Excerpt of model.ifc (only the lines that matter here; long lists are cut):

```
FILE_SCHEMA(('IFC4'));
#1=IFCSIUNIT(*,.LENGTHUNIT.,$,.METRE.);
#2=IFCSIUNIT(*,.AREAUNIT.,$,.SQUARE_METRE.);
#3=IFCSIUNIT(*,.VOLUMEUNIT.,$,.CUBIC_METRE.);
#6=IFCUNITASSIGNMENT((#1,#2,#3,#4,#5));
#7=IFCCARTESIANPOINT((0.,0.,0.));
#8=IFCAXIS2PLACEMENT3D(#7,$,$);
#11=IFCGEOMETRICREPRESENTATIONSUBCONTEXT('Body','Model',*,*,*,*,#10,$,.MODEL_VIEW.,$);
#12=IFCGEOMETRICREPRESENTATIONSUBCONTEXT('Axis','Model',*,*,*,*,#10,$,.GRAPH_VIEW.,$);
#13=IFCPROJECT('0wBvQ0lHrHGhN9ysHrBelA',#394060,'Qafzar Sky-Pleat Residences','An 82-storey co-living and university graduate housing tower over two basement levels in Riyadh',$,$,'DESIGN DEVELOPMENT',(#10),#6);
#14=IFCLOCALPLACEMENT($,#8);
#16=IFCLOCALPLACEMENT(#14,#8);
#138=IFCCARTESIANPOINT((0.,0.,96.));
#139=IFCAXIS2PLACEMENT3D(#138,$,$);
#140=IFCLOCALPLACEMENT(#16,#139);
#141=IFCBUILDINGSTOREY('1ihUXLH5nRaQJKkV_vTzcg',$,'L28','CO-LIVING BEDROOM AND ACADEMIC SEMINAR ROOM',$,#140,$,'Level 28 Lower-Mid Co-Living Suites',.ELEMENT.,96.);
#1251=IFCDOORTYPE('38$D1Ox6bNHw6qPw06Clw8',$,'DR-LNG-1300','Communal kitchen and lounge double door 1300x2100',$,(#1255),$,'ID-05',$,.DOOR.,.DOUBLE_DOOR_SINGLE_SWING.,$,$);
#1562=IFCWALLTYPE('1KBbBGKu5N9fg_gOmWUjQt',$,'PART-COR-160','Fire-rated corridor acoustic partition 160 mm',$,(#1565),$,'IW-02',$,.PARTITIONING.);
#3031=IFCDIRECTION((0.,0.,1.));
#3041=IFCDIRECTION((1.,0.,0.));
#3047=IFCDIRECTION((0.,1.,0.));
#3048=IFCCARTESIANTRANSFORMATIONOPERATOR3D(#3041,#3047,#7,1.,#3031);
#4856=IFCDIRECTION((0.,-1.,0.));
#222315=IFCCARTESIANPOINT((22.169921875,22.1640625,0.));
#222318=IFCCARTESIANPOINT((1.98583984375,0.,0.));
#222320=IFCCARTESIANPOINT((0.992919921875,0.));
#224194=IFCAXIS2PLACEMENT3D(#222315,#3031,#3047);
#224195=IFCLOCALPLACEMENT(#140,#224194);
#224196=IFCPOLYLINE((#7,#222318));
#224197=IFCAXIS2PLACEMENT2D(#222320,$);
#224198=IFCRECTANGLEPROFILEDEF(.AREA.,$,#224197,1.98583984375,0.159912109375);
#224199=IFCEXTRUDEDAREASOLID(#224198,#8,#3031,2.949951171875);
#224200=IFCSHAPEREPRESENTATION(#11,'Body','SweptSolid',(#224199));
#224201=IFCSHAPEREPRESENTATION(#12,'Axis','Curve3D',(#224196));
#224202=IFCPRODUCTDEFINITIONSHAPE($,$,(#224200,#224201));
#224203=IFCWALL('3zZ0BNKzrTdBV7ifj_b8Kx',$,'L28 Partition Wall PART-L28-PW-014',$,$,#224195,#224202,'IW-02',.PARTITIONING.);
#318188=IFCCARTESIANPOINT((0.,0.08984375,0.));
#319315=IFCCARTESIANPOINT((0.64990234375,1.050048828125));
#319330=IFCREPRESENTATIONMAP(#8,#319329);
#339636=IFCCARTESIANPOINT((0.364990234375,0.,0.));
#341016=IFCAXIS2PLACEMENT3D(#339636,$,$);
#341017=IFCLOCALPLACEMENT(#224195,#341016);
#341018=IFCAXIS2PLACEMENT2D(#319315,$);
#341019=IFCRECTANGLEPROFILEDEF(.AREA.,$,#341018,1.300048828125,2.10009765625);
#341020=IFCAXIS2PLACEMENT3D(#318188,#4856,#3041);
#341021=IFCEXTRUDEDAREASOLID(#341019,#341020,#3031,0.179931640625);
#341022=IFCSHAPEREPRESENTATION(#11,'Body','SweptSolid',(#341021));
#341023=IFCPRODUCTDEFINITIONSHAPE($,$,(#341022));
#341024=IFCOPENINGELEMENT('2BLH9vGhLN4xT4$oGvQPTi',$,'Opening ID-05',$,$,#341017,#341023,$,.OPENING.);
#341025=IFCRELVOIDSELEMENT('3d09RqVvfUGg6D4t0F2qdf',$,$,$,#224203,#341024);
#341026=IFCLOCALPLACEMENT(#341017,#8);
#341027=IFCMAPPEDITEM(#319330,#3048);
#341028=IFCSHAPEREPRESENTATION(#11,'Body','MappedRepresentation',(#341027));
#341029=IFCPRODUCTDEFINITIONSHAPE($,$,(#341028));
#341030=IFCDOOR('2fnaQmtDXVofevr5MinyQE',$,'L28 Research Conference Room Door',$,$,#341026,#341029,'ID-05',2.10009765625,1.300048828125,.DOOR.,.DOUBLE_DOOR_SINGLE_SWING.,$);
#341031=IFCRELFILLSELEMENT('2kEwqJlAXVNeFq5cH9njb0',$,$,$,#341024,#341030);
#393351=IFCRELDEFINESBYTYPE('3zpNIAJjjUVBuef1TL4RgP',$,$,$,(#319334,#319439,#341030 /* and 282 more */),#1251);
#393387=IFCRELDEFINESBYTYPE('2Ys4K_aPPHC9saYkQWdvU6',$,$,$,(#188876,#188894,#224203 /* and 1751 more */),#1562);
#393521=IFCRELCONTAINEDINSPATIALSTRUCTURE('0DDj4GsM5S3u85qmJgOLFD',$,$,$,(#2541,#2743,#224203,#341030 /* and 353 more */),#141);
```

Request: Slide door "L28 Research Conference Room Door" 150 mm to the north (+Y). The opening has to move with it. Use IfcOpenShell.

```python
import ifcopenshell
import ifcopenshell.api.geometry
import ifcopenshell.util.placement

model = ifcopenshell.open("model.ifc")

door = model.by_id(341030)
opening = door.FillsVoids[0].RelatingOpeningElement
wall = opening.VoidsElements[0].RelatingBuildingElement

wall_matrix = ifcopenshell.util.placement.get_local_placement(wall.ObjectPlacement)
shift = wall_matrix[:3, 0] * 0.15
before = ifcopenshell.util.placement.get_local_placement(door.ObjectPlacement)[:3, 3].copy()

# The door is placed relative to its opening, so it follows when the opening moves.
matrix = ifcopenshell.util.placement.get_local_placement(opening.ObjectPlacement)
matrix[:3, 3] += shift
ifcopenshell.api.geometry.edit_object_placement(
    model, product=opening, matrix=matrix, is_si=False, should_transform_children=True
)

after = ifcopenshell.util.placement.get_local_placement(door.ObjectPlacement)[:3, 3]
print("door moved by", (after - before).round(3) + 0.0)

model.write("model_v2.ifc")
```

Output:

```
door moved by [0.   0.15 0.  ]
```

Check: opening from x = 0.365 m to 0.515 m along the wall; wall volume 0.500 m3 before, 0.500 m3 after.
